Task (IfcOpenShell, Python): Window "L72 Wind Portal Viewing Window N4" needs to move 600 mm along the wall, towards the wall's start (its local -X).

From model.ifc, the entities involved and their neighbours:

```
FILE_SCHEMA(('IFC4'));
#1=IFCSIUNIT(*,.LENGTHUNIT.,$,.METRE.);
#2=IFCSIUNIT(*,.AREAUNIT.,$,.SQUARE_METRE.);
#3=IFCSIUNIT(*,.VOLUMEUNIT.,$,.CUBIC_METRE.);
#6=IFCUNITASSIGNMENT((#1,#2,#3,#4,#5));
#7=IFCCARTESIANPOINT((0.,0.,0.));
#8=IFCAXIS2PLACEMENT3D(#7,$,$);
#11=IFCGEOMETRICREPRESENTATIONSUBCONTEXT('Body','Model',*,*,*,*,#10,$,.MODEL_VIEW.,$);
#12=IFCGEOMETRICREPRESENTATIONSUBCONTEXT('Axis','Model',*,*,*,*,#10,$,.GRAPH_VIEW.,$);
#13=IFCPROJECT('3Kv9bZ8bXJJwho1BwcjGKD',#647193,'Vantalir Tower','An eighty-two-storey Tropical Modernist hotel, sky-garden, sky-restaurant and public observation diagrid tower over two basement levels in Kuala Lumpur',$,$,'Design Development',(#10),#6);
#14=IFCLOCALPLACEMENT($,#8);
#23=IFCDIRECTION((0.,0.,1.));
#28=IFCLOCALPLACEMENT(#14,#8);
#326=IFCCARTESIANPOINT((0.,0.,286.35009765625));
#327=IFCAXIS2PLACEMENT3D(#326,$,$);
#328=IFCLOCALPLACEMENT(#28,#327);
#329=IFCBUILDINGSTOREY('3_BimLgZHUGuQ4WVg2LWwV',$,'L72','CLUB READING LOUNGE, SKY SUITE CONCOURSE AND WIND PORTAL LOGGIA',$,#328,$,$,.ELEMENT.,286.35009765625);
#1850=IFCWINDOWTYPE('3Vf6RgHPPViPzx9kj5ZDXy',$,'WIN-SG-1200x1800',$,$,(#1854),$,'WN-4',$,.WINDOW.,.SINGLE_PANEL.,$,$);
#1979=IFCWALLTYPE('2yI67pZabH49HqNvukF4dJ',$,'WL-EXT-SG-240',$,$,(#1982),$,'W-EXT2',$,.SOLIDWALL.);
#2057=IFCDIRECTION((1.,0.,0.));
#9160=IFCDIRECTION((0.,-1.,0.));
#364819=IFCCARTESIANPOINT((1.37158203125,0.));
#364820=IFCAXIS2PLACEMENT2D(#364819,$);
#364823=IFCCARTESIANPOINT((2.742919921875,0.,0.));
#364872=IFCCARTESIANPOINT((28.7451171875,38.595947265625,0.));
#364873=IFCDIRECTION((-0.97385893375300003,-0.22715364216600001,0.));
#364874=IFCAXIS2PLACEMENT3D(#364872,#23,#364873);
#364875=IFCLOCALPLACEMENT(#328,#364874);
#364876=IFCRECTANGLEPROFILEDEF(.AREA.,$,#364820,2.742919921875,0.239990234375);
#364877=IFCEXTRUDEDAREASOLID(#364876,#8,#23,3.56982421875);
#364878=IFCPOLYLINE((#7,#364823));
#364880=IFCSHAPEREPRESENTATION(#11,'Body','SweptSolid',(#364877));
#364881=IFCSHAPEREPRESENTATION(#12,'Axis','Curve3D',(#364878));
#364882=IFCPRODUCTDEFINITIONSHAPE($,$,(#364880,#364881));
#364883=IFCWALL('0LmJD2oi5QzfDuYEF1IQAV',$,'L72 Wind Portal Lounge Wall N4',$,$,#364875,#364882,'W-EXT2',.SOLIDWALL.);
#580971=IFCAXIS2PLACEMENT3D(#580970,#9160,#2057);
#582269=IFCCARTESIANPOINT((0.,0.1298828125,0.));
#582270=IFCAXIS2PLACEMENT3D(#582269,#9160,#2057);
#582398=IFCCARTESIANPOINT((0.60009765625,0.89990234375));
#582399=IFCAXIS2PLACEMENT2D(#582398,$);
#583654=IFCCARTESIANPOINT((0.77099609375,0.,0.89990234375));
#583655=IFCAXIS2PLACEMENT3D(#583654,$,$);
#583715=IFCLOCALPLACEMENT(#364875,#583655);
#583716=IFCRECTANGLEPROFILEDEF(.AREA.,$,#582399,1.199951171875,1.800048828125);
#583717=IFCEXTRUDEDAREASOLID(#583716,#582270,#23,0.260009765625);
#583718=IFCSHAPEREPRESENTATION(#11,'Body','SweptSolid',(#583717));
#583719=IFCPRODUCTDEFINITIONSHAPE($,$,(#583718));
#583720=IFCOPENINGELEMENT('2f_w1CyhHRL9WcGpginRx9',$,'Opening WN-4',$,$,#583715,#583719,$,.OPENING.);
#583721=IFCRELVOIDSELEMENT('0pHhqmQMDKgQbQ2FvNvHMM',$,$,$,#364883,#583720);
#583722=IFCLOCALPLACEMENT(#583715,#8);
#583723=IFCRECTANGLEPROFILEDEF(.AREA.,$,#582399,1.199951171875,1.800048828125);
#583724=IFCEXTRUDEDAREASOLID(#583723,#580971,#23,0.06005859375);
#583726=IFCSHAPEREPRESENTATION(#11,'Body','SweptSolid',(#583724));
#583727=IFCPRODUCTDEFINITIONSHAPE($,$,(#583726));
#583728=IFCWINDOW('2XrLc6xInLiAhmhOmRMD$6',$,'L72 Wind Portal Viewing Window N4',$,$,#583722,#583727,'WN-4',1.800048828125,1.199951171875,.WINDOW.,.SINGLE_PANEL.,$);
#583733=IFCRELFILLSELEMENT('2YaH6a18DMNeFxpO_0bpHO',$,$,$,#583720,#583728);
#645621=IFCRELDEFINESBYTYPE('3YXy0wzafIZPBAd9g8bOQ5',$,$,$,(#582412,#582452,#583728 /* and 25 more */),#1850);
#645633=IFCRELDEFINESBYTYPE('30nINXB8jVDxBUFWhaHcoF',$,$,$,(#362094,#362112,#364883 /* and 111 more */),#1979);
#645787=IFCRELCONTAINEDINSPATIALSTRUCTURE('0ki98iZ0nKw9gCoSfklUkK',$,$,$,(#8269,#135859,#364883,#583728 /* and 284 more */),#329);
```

```python
import ifcopenshell
import ifcopenshell.api.geometry
import ifcopenshell.util.placement
import ifcopenshell.util.unit

model = ifcopenshell.open("model.ifc")
unit_scale = ifcopenshell.util.unit.calculate_unit_scale(model)

window = model.by_id(583728)
opening = window.FillsVoids[0].RelatingOpeningElement
wall = opening.VoidsElements[0].RelatingBuildingElement

wall_matrix = ifcopenshell.util.placement.get_local_placement(wall.ObjectPlacement)
shift = wall_matrix[:3, 0] * -0.6 / unit_scale
before = ifcopenshell.util.placement.get_local_placement(window.ObjectPlacement)[:3, 3].copy()

# The window is placed relative to its opening, so it follows when the opening moves.
matrix = ifcopenshell.util.placement.get_local_placement(opening.ObjectPlacement)
matrix[:3, 3] += shift
ifcopenshell.api.geometry.edit_object_placement(
    model, product=opening, matrix=matrix, is_si=False, should_transform_children=True
)

after = ifcopenshell.util.placement.get_local_placement(window.ObjectPlacement)[:3, 3]
print("window moved by", (after - before).round(3) + 0.0)

model.write("model_rev.ifc")
```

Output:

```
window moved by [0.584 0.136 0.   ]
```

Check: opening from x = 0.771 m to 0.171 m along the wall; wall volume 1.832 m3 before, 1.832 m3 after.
